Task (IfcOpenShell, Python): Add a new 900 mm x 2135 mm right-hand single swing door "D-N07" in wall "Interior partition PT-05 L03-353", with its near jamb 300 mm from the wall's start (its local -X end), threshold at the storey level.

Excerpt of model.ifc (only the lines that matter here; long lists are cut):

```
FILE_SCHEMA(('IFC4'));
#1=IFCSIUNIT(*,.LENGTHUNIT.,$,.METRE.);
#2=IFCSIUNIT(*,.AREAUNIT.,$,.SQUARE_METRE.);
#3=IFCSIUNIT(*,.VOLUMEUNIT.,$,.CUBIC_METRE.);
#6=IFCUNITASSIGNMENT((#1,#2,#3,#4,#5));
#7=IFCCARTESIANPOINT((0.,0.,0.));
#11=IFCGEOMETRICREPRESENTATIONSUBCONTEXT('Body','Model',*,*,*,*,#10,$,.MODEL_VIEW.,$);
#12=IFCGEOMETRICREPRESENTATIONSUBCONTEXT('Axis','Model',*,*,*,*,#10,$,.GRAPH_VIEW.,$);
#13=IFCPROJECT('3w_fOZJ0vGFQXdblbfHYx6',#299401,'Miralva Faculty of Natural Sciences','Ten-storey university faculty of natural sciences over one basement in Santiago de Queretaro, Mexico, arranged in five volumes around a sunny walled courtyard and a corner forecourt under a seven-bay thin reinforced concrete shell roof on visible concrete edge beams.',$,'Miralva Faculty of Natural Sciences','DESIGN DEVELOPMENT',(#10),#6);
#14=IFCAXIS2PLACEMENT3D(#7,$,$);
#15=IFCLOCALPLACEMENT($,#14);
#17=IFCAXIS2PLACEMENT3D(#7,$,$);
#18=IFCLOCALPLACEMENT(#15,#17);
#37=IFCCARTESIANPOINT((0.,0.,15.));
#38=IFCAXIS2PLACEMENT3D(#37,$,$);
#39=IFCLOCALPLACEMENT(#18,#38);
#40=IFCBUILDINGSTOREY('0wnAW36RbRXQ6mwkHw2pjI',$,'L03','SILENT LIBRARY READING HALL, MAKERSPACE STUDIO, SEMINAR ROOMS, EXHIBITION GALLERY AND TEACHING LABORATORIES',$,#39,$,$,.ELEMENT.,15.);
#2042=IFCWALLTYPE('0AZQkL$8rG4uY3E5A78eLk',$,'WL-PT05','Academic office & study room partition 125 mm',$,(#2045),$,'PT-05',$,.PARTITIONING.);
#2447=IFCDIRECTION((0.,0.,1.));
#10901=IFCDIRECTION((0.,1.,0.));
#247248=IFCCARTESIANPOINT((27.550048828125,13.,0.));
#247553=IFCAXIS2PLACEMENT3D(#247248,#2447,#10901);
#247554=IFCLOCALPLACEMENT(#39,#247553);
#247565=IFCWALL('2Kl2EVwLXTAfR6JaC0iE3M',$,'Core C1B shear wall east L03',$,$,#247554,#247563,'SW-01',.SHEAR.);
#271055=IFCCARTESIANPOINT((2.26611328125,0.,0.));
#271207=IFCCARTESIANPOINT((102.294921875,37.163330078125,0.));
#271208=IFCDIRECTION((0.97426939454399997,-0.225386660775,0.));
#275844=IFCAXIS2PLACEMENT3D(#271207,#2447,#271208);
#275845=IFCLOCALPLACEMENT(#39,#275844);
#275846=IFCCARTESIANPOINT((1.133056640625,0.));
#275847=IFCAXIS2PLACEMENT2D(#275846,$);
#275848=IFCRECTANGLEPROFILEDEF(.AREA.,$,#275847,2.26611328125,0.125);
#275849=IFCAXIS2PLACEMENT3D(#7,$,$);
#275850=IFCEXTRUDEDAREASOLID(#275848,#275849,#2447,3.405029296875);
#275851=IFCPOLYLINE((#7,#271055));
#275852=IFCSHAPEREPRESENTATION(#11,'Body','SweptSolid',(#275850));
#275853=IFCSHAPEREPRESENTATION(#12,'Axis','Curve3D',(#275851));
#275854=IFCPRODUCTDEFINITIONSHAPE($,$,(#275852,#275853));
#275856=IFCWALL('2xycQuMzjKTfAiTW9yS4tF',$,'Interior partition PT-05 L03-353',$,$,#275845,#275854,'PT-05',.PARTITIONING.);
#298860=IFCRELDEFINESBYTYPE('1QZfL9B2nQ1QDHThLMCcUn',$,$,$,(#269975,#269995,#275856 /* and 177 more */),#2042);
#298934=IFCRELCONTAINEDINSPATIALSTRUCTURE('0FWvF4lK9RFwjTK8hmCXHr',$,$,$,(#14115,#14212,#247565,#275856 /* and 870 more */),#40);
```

```python
import numpy as np
import ifcopenshell
import ifcopenshell.api.feature
import ifcopenshell.api.geometry
import ifcopenshell.api.root
import ifcopenshell.api.spatial
import ifcopenshell.geom
import ifcopenshell.util.element
import ifcopenshell.util.placement
import ifcopenshell.util.representation
import ifcopenshell.util.shape
import ifcopenshell.util.unit

model = ifcopenshell.open("model.ifc")
unit_scale = ifcopenshell.util.unit.calculate_unit_scale(model)
settings = ifcopenshell.geom.settings()


def volume(element):
    """Net volume in cubic metres, openings subtracted."""
    shape = ifcopenshell.geom.create_shape(settings, element)
    return ifcopenshell.util.shape.get_volume(shape.geometry)


wall = model.by_guid("2xycQuMzjKTfAiTW9yS4tF")
storey = ifcopenshell.util.element.get_container(wall, ifc_class="IfcBuildingStorey")
context = ifcopenshell.util.representation.get_context(model, "Model", "Body", "MODEL_VIEW")
before = volume(wall)

width, height, from_end, sill = 0.9, 2.135, 0.3, 0.0  # metres

# The wall runs along its own X axis, and the end named is its -X end.
wall_shape = ifcopenshell.geom.create_shape(settings, wall)
x, y, z = ifcopenshell.util.shape.get_vertices(wall_shape.geometry).T
start = x.min() + from_end
face, thickness = float(y.min()), float(y.max() - y.min())
wall_matrix = ifcopenshell.util.placement.get_local_placement(wall.ObjectPlacement)
level = ifcopenshell.util.placement.get_local_placement(storey.ObjectPlacement)[2, 3]


def in_wall(x, y):
    """Placement at x, y metres in the wall's axes, at sill height."""
    matrix = wall_matrix.copy()
    matrix[:, 3] = wall_matrix @ np.array([x / unit_scale, y / unit_scale, 0.0, 1.0])
    matrix[2, 3] = level + sill / unit_scale
    return matrix


# Opening: a box that overshoots both wall faces by 50 mm.
opening = ifcopenshell.api.root.create_entity(model, ifc_class="IfcOpeningElement", predefined_type="OPENING")
box = ifcopenshell.api.geometry.add_wall_representation(
    model, context=context, length=width, height=height, thickness=thickness + 0.1
)
ifcopenshell.api.geometry.assign_representation(model, product=opening, representation=box)
ifcopenshell.api.geometry.edit_object_placement(model, product=opening, matrix=in_wall(start, face - 0.05), is_si=False)
ifcopenshell.api.feature.add_feature(model, feature=opening, element=wall)

door = ifcopenshell.api.root.create_entity(model, ifc_class="IfcDoor", name="D-N07", predefined_type="DOOR")
door.OverallWidth, door.OverallHeight = width / unit_scale, height / unit_scale
door.OperationType = "SINGLE_SWING_RIGHT"
body = ifcopenshell.api.geometry.add_door_representation(
    model,
    context=context,
    overall_width=door.OverallWidth,
    overall_height=door.OverallHeight,
    operation_type="SINGLE_SWING_RIGHT",
    lining_properties={"LiningDepth": thickness / unit_scale, "ThresholdDepth": thickness / unit_scale},
)
ifcopenshell.api.geometry.assign_representation(model, product=door, representation=body)
ifcopenshell.api.spatial.assign_container(model, products=[door], relating_structure=storey)
ifcopenshell.api.feature.add_filling(model, opening=opening, element=door)

# The lining spans the wall, so the door starts at the wall face.
ifcopenshell.api.geometry.edit_object_placement(model, product=door, matrix=in_wall(start, face), is_si=False)

after = volume(wall)

print(f"wall volume {before:.3f} -> {after:.3f} m3")

model.write("model_v2.ifc")
```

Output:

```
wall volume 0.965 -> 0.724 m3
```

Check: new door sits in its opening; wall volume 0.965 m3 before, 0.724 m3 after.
